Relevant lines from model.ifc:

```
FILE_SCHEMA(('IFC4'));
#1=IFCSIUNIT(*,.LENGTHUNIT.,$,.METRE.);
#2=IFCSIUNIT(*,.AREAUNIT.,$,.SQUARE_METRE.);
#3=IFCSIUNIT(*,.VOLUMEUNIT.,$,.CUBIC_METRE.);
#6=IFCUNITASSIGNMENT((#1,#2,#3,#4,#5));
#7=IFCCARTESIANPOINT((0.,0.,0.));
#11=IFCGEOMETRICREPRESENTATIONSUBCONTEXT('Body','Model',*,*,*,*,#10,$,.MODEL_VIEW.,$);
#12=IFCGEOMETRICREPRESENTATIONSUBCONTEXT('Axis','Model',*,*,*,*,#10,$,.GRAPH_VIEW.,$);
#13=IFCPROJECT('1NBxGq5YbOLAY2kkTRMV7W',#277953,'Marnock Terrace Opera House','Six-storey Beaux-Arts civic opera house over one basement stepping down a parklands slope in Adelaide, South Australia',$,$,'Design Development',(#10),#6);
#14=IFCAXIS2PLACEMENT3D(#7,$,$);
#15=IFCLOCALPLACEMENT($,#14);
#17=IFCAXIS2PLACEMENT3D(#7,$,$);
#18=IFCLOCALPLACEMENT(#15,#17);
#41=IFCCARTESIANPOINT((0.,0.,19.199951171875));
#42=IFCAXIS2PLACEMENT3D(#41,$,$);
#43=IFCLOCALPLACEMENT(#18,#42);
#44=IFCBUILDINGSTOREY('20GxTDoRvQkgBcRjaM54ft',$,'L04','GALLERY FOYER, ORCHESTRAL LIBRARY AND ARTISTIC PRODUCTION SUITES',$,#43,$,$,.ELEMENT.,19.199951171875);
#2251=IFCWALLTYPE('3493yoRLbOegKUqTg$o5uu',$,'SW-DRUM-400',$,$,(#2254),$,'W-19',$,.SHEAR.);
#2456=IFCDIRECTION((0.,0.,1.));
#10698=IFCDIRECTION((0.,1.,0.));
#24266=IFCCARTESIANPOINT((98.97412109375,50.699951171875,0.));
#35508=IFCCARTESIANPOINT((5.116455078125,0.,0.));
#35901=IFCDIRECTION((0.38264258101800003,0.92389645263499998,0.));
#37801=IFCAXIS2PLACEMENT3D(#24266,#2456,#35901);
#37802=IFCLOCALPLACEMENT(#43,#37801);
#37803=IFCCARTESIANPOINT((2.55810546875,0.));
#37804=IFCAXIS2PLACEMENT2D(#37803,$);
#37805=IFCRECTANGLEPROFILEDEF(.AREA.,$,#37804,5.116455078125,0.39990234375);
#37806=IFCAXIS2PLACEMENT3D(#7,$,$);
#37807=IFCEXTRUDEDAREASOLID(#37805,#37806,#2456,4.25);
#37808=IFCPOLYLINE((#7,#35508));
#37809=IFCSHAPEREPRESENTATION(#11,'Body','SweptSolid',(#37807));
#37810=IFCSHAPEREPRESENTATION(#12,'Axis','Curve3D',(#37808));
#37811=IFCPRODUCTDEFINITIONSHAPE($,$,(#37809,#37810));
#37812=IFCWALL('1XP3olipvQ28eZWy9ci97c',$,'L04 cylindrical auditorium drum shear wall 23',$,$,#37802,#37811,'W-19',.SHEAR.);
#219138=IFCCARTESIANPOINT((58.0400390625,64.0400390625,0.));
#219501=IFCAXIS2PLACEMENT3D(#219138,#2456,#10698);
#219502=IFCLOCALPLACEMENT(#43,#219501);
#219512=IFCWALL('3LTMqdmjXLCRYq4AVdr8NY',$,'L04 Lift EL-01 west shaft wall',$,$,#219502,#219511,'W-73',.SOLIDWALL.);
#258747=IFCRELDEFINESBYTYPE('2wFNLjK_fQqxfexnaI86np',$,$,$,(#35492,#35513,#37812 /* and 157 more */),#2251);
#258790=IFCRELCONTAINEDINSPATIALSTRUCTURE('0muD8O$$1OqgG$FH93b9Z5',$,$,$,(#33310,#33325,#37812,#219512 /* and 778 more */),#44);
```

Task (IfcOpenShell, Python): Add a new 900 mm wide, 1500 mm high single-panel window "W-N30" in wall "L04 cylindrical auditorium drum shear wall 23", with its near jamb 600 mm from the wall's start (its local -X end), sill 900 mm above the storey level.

```python
import numpy as np
import ifcopenshell
import ifcopenshell.api.feature
import ifcopenshell.api.geometry
import ifcopenshell.api.root
import ifcopenshell.api.spatial
import ifcopenshell.geom
import ifcopenshell.util.element
import ifcopenshell.util.placement
import ifcopenshell.util.representation
import ifcopenshell.util.shape
import ifcopenshell.util.unit

model = ifcopenshell.open("model.ifc")
unit_scale = ifcopenshell.util.unit.calculate_unit_scale(model)
settings = ifcopenshell.geom.settings()


def volume(element):
    """Net volume in cubic metres, openings subtracted."""
    shape = ifcopenshell.geom.create_shape(settings, element)
    return ifcopenshell.util.shape.get_volume(shape.geometry)


wall = model.by_guid("1XP3olipvQ28eZWy9ci97c")
storey = ifcopenshell.util.element.get_container(wall, ifc_class="IfcBuildingStorey")
context = ifcopenshell.util.representation.get_context(model, "Model", "Body", "MODEL_VIEW")
before = volume(wall)

width, height, from_end, sill = 0.9, 1.5, 0.6, 0.9  # metres

# The wall runs along its own X axis, and the end named is its -X end.
wall_shape = ifcopenshell.geom.create_shape(settings, wall)
x, y, z = ifcopenshell.util.shape.get_vertices(wall_shape.geometry).T
start = x.min() + from_end
face, thickness = float(y.min()), float(y.max() - y.min())
wall_matrix = ifcopenshell.util.placement.get_local_placement(wall.ObjectPlacement)
level = ifcopenshell.util.placement.get_local_placement(storey.ObjectPlacement)[2, 3]


def in_wall(x, y):
    """Placement at x, y metres in the wall's axes, at sill height."""
    matrix = wall_matrix.copy()
    matrix[:, 3] = wall_matrix @ np.array([x / unit_scale, y / unit_scale, 0.0, 1.0])
    matrix[2, 3] = level + sill / unit_scale
    return matrix


# Opening: a box that overshoots both wall faces by 50 mm.
opening = ifcopenshell.api.root.create_entity(model, ifc_class="IfcOpeningElement", predefined_type="OPENING")
box = ifcopenshell.api.geometry.add_wall_representation(
    model, context=context, length=width, height=height, thickness=thickness + 0.1
)
ifcopenshell.api.geometry.assign_representation(model, product=opening, representation=box)
ifcopenshell.api.geometry.edit_object_placement(model, product=opening, matrix=in_wall(start, face - 0.05), is_si=False)
ifcopenshell.api.feature.add_feature(model, feature=opening, element=wall)

window = ifcopenshell.api.root.create_entity(model, ifc_class="IfcWindow", name="W-N30", predefined_type="WINDOW")
window.OverallWidth, window.OverallHeight = width / unit_scale, height / unit_scale
window.PartitioningType = "SINGLE_PANEL"
body = ifcopenshell.api.geometry.add_window_representation(
    model,
    context=context,
    overall_width=window.OverallWidth,
    overall_height=window.OverallHeight,
    partition_type="SINGLE_PANEL",
)
ifcopenshell.api.geometry.assign_representation(model, product=window, representation=body)
ifcopenshell.api.spatial.assign_container(model, products=[window], relating_structure=storey)
ifcopenshell.api.feature.add_filling(model, opening=opening, element=window)

# Centre the window in the wall's thickness.
ifcopenshell.api.geometry.edit_object_placement(model, product=window, matrix=in_wall(start, face), is_si=False)
window_shape = ifcopenshell.geom.create_shape(settings, window)
depth = ifcopenshell.util.shape.get_vertices(window_shape.geometry)[:, 1]
offset = face + thickness / 2 - (depth.min() + depth.max()) / 2
ifcopenshell.api.geometry.edit_object_placement(model, product=window, matrix=in_wall(start, offset), is_si=False)

after = volume(wall)

print(f"wall volume {before:.3f} -> {after:.3f} m3")

model.write("model_v2.ifc")
```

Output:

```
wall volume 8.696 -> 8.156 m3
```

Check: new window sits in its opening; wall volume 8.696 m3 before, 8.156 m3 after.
